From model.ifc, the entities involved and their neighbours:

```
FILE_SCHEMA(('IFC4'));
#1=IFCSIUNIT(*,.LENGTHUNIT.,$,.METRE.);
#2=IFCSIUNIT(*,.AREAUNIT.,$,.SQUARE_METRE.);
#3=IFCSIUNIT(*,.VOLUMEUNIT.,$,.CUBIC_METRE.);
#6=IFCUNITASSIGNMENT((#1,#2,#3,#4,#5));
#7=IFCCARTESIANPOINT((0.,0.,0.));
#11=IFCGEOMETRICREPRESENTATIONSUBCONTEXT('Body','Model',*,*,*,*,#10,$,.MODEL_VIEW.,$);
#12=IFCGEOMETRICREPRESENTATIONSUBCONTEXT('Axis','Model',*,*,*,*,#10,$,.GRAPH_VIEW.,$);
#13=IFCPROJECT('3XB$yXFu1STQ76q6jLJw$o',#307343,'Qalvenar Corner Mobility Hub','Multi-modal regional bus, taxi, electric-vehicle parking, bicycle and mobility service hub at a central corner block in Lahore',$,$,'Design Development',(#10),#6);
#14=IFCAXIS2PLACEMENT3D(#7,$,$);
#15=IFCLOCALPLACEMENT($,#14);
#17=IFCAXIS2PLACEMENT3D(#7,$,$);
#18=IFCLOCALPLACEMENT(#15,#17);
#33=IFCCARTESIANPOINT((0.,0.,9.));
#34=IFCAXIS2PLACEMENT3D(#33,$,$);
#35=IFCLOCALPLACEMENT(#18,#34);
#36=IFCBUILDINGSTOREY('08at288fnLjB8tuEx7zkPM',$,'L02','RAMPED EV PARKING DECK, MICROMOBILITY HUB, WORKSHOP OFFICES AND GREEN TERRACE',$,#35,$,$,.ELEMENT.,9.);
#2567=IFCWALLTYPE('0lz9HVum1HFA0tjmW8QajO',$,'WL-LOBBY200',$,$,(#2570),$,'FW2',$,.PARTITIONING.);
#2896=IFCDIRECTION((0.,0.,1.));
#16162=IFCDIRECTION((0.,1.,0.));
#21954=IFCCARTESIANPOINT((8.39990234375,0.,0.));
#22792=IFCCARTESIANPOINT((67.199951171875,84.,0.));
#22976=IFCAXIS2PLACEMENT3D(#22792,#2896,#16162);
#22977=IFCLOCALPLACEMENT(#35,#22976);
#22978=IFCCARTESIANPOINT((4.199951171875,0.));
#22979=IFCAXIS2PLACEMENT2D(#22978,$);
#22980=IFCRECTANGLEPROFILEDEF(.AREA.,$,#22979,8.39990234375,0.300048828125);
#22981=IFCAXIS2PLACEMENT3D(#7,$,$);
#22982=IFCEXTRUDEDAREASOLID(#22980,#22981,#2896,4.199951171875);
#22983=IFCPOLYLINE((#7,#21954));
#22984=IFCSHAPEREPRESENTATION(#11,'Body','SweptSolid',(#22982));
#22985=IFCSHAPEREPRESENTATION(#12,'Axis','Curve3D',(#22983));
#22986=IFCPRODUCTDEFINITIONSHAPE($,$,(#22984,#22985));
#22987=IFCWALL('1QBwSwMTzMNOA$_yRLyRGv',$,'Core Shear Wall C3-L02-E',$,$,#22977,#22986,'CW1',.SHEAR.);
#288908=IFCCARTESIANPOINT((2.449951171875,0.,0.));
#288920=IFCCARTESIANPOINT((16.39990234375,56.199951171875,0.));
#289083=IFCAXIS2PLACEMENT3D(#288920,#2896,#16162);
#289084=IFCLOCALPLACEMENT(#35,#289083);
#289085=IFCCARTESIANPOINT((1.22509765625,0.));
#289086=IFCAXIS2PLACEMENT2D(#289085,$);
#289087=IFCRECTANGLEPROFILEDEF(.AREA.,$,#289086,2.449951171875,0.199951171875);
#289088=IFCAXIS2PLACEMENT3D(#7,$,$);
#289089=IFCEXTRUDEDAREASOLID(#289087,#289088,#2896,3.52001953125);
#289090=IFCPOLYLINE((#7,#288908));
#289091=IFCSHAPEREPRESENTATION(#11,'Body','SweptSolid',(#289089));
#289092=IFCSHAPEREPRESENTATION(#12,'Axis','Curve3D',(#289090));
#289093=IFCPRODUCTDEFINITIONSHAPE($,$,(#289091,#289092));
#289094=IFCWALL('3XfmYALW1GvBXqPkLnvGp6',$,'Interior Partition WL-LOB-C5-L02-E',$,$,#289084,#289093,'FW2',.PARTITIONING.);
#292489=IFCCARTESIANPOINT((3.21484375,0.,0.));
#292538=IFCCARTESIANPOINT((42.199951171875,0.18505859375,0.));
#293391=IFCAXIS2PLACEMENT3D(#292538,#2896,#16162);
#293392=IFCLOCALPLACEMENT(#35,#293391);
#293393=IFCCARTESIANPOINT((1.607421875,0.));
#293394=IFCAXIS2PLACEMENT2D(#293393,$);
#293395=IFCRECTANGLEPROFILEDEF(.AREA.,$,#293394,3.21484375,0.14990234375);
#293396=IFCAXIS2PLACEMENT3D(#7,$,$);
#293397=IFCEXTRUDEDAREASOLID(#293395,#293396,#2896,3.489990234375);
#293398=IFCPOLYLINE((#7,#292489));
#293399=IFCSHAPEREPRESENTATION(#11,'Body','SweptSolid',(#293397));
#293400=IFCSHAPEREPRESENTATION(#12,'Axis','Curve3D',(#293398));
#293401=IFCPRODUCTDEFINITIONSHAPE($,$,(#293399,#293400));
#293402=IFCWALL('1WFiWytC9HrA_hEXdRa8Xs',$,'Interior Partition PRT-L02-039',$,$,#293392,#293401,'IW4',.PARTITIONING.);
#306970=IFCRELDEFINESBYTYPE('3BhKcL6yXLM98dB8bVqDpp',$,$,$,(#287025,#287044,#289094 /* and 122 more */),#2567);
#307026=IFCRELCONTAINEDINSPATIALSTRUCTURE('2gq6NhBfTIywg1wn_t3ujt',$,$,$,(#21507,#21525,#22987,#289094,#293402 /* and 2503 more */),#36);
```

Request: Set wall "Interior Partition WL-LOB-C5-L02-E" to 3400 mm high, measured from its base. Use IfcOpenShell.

```python
import ifcopenshell
import ifcopenshell.geom
import ifcopenshell.util.representation
import ifcopenshell.util.shape
import ifcopenshell.util.unit

model = ifcopenshell.open("model.ifc")
unit_scale = ifcopenshell.util.unit.calculate_unit_scale(model)
settings = ifcopenshell.geom.settings()


def volume(element):
    """Net volume in cubic metres, openings subtracted."""
    shape = ifcopenshell.geom.create_shape(settings, element)
    return ifcopenshell.util.shape.get_volume(shape.geometry)


wall = model.by_guid("3XfmYALW1GvBXqPkLnvGp6")
before = volume(wall)

body = ifcopenshell.util.representation.get_representation(wall, "Model", "Body")
solid = body.Items[0]
old_height = solid.Depth
solid.Depth = 3.4 / unit_scale
after = volume(wall)

print(f"height {old_height:g} -> {solid.Depth:g}, volume {before:.3f} -> {after:.3f} m3")

model.write("model_updated.ifc")
```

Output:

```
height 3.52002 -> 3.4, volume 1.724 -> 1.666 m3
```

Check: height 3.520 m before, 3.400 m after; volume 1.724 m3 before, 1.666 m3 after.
